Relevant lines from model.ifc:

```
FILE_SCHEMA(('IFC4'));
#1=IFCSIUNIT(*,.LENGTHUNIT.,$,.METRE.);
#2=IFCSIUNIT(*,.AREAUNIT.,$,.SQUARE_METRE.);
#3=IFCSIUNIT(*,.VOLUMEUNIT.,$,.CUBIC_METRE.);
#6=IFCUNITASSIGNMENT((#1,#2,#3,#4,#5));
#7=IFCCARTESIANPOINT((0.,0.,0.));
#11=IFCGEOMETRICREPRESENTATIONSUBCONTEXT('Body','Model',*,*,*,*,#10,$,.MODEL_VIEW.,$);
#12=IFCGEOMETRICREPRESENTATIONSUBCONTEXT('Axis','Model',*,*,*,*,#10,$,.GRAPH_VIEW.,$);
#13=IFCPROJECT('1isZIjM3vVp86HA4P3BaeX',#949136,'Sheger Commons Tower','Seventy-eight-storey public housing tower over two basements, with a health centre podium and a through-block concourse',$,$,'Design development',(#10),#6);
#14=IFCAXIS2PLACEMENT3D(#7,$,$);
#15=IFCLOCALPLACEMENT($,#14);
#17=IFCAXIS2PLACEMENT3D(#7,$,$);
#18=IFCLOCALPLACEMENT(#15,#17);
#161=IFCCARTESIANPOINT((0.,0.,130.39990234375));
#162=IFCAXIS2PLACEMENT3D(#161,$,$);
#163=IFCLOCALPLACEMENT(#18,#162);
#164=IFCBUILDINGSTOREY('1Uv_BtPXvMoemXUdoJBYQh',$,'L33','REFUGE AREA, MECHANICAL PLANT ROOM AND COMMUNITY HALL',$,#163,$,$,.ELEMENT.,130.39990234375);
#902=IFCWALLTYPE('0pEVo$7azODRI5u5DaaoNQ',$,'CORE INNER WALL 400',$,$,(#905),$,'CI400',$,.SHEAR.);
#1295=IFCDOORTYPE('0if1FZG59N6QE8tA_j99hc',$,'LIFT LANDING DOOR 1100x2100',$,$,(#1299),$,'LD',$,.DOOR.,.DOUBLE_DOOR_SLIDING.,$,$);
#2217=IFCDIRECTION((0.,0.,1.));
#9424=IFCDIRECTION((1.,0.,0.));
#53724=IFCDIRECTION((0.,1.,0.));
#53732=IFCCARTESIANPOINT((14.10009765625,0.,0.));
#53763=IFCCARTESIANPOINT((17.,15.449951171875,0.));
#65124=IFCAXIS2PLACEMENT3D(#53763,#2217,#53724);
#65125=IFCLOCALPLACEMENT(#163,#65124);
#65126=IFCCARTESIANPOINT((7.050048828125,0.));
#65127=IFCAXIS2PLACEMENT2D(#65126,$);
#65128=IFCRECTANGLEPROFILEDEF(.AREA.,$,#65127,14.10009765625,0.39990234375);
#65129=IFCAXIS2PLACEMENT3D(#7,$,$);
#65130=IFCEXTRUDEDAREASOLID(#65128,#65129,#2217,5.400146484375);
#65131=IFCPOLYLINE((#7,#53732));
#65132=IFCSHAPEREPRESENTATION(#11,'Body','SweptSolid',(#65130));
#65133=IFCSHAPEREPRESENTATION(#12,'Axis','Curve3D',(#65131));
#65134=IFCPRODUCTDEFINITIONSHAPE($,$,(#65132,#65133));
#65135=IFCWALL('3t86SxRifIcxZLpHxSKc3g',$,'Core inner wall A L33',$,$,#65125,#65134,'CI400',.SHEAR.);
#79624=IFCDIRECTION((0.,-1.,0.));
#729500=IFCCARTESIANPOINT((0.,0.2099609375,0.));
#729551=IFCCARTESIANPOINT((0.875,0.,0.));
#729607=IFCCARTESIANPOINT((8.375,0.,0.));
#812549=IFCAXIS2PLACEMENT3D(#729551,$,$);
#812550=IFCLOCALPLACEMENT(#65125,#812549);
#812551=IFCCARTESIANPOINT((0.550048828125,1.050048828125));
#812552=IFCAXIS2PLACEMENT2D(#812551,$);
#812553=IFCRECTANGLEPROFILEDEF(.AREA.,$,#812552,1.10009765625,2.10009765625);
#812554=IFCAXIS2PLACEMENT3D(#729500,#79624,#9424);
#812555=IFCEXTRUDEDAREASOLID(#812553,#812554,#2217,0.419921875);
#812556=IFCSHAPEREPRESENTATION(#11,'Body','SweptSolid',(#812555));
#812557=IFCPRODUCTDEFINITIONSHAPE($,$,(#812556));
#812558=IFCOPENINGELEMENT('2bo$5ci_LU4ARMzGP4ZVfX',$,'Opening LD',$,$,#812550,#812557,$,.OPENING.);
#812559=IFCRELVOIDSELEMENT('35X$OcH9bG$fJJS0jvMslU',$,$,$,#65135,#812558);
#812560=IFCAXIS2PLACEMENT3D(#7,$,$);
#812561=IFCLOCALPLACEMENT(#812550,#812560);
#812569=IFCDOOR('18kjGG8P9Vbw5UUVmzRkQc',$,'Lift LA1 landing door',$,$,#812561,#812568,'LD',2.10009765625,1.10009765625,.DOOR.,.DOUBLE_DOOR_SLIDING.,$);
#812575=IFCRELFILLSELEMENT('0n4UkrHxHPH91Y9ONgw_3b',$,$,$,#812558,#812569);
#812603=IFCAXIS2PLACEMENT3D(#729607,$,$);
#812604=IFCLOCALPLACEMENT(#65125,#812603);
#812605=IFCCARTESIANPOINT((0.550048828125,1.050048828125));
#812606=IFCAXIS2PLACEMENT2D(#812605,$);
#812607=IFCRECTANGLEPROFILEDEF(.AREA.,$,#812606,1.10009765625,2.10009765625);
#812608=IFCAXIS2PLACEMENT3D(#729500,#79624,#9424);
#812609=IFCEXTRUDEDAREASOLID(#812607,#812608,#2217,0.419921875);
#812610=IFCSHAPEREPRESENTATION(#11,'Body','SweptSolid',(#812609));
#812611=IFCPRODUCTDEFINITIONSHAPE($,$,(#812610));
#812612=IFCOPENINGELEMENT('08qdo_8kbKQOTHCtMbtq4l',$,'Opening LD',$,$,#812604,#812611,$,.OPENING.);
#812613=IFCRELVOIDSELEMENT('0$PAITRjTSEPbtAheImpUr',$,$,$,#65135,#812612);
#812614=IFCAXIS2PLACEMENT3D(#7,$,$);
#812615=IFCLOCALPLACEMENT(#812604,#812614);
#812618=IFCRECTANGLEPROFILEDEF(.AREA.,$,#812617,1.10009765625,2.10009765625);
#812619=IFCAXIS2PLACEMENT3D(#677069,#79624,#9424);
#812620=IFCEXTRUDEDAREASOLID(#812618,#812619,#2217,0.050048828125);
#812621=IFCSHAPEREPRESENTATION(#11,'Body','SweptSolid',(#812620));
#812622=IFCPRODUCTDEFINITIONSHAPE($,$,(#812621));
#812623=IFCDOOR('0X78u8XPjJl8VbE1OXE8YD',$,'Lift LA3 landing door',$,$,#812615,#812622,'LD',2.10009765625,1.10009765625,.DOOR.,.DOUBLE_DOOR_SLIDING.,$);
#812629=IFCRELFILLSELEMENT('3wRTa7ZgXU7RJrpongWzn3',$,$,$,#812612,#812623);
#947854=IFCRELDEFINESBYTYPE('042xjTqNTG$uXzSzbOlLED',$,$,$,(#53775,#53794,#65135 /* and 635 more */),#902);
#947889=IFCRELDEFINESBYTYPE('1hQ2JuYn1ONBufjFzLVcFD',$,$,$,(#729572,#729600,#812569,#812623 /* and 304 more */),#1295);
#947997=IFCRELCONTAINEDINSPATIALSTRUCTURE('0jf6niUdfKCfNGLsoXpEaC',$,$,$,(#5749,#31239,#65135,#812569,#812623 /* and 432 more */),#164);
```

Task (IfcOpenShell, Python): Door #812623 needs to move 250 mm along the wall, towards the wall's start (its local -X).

```python
import ifcopenshell
import ifcopenshell.api.geometry
import ifcopenshell.util.placement

model = ifcopenshell.open("model.ifc")

door = model.by_guid("0X78u8XPjJl8VbE1OXE8YD")
opening = door.FillsVoids[0].RelatingOpeningElement
wall = opening.VoidsElements[0].RelatingBuildingElement

wall_matrix = ifcopenshell.util.placement.get_local_placement(wall.ObjectPlacement)
shift = wall_matrix[:3, 0] * -0.25
before = ifcopenshell.util.placement.get_local_placement(door.ObjectPlacement)[:3, 3].copy()

# The door is placed relative to its opening, so it follows when the opening moves.
matrix = ifcopenshell.util.placement.get_local_placement(opening.ObjectPlacement)
matrix[:3, 3] += shift
ifcopenshell.api.geometry.edit_object_placement(
    model, product=opening, matrix=matrix, is_si=False, should_transform_children=True
)

after = ifcopenshell.util.placement.get_local_placement(door.ObjectPlacement)[:3, 3]
print("door moved by", (after - before).round(3) + 0.0)

model.write("model_v2.ifc")
```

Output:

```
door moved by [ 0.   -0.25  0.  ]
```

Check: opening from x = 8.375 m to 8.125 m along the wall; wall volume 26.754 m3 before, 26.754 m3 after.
